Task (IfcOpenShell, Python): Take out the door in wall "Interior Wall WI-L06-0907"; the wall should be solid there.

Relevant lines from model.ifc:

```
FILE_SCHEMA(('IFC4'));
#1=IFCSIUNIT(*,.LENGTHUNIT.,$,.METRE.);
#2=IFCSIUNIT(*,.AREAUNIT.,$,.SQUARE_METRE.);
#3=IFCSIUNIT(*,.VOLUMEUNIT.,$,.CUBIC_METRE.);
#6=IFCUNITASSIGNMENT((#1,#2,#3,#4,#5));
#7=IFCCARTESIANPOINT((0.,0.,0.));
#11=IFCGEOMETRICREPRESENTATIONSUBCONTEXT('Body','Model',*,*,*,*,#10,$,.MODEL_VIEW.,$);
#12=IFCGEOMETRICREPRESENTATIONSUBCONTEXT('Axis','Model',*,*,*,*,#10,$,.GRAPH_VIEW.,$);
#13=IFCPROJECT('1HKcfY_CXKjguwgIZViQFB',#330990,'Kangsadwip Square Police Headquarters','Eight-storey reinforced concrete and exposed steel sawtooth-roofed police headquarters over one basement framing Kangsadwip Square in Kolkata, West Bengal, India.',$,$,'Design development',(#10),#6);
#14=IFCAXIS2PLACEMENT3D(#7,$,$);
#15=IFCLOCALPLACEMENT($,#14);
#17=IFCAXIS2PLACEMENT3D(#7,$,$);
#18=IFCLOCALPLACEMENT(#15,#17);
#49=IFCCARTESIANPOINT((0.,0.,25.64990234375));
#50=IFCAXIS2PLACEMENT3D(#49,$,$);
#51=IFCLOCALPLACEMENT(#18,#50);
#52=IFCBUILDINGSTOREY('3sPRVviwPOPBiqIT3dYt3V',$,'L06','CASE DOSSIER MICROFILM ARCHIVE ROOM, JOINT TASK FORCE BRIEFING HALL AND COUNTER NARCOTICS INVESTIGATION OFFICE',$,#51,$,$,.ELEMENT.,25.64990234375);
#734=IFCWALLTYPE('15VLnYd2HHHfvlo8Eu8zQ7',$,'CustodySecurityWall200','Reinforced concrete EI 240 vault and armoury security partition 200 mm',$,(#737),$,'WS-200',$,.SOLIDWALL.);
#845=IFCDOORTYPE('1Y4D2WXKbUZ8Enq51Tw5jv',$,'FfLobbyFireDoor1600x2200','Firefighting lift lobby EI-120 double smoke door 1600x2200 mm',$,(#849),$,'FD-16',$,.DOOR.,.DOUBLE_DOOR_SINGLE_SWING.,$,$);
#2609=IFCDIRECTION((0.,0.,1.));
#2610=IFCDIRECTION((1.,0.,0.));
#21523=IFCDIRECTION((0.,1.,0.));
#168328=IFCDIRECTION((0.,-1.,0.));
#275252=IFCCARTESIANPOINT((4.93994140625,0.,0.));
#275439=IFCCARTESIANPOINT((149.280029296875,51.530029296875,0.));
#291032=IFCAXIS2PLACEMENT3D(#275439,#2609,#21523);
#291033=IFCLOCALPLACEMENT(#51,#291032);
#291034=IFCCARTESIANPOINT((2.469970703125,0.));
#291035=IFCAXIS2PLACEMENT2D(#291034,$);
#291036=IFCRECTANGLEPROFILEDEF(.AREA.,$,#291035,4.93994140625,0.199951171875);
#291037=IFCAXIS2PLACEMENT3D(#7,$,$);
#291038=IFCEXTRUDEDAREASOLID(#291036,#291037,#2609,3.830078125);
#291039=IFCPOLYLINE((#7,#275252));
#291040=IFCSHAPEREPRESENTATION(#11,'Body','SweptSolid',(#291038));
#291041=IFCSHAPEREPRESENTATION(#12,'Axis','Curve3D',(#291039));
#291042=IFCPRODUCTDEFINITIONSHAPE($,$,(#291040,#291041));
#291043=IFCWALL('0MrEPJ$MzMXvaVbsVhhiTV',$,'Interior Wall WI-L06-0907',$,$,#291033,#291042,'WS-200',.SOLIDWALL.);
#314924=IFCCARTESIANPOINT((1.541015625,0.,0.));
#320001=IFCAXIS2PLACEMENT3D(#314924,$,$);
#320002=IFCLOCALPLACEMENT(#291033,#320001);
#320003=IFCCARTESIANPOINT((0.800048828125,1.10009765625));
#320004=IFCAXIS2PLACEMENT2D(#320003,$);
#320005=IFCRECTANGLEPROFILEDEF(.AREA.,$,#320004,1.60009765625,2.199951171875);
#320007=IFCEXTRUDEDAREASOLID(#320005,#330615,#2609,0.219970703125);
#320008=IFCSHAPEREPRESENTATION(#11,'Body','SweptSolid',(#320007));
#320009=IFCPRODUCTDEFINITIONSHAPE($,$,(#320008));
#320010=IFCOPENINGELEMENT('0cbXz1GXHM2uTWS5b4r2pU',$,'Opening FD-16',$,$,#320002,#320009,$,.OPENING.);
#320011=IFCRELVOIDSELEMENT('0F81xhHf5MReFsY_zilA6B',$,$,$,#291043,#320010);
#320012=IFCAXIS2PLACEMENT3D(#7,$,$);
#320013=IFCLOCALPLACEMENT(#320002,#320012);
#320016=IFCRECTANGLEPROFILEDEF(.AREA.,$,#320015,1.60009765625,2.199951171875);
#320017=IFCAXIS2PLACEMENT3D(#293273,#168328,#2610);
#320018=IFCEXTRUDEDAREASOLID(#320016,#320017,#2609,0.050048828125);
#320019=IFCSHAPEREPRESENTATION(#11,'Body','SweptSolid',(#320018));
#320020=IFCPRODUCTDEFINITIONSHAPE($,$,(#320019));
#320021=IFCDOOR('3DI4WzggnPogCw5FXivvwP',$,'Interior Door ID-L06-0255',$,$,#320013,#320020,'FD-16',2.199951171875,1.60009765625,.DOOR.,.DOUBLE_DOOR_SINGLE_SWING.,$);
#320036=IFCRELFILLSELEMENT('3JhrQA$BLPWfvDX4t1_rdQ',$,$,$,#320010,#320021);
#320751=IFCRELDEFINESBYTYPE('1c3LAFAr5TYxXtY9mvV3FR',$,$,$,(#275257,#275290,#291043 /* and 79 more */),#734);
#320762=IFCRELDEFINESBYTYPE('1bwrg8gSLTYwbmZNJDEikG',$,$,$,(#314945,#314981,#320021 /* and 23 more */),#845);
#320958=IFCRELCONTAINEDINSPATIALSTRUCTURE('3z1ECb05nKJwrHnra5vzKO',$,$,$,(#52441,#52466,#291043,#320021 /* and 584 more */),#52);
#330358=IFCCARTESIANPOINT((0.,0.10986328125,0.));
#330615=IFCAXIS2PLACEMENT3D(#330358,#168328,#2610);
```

```python
import ifcopenshell
import ifcopenshell.api.feature
import ifcopenshell.api.root
import ifcopenshell.geom
import ifcopenshell.util.shape

model = ifcopenshell.open("model.ifc")
settings = ifcopenshell.geom.settings()


def volume(element):
    """Net volume in cubic metres, openings subtracted."""
    shape = ifcopenshell.geom.create_shape(settings, element)
    return ifcopenshell.util.shape.get_volume(shape.geometry)


door = model.by_guid("3DI4WzggnPogCw5FXivvwP")
opening = door.FillsVoids[0].RelatingOpeningElement
wall = opening.VoidsElements[0].RelatingBuildingElement
before = volume(wall)

ifcopenshell.api.root.remove_product(model, product=door)
ifcopenshell.api.feature.remove_feature(model, feature=opening)

after = volume(wall)

print(f"wall volume {before:.3f} -> {after:.3f} m3")

model.write("model_rev.ifc")
```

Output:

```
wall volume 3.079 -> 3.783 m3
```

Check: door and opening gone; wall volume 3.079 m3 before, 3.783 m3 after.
